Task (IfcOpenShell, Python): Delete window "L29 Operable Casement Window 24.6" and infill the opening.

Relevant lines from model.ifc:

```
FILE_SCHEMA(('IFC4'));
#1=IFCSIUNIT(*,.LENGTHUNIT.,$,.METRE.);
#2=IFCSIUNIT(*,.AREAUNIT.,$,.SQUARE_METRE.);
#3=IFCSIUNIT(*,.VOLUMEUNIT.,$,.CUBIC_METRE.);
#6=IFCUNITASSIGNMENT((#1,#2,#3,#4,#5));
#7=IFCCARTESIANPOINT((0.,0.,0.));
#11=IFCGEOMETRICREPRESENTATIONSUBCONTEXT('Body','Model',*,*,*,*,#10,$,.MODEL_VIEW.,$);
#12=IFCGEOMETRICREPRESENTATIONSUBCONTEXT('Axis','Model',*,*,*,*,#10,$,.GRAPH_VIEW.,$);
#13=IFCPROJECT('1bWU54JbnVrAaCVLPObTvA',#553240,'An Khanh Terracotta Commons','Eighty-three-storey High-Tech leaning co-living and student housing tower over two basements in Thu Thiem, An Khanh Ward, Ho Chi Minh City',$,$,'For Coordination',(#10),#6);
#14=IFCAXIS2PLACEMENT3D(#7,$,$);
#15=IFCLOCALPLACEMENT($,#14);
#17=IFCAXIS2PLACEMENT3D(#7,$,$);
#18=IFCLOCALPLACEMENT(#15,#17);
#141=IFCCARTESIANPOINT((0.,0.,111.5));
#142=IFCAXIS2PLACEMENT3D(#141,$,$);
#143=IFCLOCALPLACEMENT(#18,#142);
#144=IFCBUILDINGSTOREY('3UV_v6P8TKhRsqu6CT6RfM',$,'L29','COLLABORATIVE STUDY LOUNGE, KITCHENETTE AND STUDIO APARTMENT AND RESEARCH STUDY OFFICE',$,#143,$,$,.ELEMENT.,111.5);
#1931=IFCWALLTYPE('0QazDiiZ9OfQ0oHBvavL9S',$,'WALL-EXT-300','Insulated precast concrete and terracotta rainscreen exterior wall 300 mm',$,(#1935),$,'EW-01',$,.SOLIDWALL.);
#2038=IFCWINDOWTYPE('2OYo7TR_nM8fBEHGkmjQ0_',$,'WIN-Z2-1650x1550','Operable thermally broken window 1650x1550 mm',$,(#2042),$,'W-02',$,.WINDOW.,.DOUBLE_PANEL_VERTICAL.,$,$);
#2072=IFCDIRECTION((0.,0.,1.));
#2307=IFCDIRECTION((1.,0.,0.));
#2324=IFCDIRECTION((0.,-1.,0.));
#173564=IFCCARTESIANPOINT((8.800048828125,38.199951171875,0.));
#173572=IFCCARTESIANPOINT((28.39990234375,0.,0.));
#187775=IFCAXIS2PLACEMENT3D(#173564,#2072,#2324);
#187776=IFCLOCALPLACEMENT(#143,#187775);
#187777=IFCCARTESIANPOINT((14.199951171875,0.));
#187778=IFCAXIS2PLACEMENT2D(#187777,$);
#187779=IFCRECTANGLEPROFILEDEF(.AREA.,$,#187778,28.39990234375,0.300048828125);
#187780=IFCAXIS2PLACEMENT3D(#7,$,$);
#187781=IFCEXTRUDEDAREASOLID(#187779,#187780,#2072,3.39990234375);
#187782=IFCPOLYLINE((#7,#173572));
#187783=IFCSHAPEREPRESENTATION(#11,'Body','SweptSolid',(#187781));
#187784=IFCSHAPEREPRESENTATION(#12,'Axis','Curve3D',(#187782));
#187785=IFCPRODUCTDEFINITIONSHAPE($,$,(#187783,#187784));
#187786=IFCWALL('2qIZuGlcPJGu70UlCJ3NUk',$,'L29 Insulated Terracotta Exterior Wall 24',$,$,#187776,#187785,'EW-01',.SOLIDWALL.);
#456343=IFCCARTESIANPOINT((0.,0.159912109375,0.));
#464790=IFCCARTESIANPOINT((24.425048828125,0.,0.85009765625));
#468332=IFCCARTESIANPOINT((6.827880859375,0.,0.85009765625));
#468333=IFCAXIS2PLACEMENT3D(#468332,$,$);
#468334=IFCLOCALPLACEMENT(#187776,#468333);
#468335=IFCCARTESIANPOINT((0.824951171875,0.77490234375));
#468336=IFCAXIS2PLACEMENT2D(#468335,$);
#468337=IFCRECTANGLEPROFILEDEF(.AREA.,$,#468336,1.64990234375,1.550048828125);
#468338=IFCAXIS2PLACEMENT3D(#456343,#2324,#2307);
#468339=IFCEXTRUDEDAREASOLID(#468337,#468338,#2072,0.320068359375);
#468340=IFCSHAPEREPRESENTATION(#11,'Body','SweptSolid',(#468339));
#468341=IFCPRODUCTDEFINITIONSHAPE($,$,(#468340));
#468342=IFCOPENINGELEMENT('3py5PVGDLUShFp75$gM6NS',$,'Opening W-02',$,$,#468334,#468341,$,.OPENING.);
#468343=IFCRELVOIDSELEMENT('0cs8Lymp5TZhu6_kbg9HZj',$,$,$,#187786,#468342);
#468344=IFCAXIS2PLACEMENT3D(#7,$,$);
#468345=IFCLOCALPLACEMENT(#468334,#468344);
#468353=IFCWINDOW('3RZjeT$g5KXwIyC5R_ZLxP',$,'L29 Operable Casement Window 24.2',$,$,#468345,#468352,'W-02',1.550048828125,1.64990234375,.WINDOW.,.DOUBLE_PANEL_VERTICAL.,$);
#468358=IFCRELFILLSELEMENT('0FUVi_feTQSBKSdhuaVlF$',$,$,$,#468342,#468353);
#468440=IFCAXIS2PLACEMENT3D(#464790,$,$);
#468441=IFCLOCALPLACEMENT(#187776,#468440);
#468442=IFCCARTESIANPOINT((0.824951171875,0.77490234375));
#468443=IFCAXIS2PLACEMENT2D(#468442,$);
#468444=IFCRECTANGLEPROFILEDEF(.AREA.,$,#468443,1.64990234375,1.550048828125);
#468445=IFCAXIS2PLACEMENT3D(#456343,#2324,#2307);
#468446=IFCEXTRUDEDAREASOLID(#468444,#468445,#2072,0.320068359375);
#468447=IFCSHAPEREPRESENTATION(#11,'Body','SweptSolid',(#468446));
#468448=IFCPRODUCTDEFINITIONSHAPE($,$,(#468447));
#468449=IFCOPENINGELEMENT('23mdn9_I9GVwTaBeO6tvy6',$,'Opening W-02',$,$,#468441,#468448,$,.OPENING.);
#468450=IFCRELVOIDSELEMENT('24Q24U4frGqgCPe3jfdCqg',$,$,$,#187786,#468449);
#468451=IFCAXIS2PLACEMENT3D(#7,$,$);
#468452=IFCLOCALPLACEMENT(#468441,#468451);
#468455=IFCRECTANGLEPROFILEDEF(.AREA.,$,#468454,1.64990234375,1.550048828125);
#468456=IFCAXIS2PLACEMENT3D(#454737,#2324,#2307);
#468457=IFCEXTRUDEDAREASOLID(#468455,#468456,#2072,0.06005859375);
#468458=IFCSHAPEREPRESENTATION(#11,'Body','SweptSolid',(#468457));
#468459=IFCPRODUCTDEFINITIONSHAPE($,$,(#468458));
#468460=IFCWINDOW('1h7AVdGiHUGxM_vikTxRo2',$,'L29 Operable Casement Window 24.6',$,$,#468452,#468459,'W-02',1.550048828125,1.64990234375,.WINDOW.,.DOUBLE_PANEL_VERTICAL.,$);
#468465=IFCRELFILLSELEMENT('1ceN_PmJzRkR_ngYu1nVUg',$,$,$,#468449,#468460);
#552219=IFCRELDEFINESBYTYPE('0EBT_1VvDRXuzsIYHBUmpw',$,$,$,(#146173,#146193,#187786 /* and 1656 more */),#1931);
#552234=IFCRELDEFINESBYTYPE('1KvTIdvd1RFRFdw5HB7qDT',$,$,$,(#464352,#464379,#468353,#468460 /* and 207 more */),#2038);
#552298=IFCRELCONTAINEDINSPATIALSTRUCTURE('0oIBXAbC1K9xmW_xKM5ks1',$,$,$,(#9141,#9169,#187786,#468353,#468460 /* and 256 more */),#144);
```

```python
import ifcopenshell
import ifcopenshell.api.feature
import ifcopenshell.api.root
import ifcopenshell.geom
import ifcopenshell.util.shape

model = ifcopenshell.open("model.ifc")
settings = ifcopenshell.geom.settings()


def volume(element):
    """Net volume in cubic metres, openings subtracted."""
    shape = ifcopenshell.geom.create_shape(settings, element)
    return ifcopenshell.util.shape.get_volume(shape.geometry)


window = model.by_guid("1h7AVdGiHUGxM_vikTxRo2")
opening = window.FillsVoids[0].RelatingOpeningElement
wall = opening.VoidsElements[0].RelatingBuildingElement
before = volume(wall)

ifcopenshell.api.root.remove_product(model, product=window)
ifcopenshell.api.feature.remove_feature(model, feature=opening)

after = volume(wall)

print(f"wall volume {before:.3f} -> {after:.3f} m3")

model.write("model_edited.ifc")
```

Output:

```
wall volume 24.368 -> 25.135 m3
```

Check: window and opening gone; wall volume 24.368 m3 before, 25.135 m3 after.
